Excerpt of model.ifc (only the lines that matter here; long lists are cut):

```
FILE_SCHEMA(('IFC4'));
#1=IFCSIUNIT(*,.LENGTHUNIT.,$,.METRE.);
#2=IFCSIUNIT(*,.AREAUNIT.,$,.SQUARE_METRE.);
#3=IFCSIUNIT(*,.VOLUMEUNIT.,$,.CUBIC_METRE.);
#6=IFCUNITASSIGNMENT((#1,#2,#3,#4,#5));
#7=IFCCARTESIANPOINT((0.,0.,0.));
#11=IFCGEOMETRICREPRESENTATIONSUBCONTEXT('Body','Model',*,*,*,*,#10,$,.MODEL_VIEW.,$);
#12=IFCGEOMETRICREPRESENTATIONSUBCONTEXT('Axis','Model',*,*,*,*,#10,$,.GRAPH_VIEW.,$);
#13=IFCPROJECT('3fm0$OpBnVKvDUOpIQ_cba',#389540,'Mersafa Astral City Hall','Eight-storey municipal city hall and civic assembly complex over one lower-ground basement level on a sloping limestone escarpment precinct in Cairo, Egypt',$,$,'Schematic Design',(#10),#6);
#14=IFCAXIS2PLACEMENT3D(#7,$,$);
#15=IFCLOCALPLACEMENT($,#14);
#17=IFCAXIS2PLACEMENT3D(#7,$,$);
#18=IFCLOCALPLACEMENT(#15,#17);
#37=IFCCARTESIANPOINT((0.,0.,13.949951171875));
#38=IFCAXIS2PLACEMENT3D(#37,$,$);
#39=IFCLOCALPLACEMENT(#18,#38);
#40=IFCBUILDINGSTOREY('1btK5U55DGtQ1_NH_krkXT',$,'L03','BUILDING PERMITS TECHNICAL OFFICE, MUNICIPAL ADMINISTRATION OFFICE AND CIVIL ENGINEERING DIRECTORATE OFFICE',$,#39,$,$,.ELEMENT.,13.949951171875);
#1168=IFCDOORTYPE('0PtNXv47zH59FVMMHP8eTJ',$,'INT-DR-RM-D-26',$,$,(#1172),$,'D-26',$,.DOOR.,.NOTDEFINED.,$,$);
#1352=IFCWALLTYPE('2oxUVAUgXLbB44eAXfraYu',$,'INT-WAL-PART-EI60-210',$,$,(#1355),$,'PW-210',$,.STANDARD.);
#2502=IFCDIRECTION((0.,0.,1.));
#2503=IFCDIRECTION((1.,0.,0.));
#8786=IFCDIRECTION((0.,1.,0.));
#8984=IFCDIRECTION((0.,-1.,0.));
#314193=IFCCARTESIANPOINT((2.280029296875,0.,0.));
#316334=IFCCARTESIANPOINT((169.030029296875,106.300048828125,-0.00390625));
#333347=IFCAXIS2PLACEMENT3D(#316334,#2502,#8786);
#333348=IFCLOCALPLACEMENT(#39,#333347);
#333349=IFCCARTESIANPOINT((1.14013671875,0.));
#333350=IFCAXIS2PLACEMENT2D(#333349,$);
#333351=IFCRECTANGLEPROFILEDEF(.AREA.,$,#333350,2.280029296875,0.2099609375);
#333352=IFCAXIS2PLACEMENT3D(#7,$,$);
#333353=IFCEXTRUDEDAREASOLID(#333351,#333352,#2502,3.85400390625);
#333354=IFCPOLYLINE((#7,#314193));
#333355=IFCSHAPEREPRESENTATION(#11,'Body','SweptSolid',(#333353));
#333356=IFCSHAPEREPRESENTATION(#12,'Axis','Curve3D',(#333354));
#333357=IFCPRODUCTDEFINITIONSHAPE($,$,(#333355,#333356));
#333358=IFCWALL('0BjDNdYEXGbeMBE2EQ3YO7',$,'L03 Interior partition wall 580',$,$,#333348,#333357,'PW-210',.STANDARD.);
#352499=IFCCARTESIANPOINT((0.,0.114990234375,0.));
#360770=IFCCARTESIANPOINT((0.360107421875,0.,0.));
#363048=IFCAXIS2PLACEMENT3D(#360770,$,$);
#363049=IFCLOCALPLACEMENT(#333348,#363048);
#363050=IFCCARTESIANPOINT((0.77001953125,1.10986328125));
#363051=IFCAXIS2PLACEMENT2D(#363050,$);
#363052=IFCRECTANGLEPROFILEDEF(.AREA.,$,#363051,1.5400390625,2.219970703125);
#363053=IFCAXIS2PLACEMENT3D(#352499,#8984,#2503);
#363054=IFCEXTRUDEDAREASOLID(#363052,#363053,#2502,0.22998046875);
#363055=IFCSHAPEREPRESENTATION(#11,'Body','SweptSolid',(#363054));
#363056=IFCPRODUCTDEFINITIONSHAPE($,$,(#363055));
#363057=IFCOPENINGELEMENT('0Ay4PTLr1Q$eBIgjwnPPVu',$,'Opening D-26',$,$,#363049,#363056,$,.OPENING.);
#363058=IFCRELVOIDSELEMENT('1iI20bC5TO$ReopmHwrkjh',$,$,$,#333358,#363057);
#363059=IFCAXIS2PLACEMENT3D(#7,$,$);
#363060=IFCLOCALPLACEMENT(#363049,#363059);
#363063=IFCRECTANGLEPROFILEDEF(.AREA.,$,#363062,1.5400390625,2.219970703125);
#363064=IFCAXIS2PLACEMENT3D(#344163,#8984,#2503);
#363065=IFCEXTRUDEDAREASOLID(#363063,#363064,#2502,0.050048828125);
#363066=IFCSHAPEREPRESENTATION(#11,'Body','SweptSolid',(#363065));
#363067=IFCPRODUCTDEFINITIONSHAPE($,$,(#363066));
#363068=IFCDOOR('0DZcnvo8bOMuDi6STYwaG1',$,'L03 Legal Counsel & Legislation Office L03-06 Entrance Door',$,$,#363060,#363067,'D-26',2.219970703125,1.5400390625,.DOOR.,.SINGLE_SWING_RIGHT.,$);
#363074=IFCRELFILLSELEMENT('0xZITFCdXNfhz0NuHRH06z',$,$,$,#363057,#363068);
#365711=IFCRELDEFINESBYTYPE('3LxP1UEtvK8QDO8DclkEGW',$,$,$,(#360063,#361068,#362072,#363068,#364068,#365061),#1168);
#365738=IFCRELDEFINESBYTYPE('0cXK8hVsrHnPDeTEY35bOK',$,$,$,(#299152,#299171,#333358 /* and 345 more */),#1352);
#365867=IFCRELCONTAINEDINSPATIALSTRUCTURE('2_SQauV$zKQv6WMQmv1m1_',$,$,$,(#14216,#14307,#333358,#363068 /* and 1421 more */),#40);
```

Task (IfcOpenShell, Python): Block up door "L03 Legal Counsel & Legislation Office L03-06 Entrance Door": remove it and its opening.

```python
import ifcopenshell
import ifcopenshell.api.feature
import ifcopenshell.api.root
import ifcopenshell.geom
import ifcopenshell.util.shape

model = ifcopenshell.open("model.ifc")
settings = ifcopenshell.geom.settings()


def volume(element):
    """Net volume in cubic metres, openings subtracted."""
    shape = ifcopenshell.geom.create_shape(settings, element)
    return ifcopenshell.util.shape.get_volume(shape.geometry)


door = model.by_guid("0DZcnvo8bOMuDi6STYwaG1")
opening = door.FillsVoids[0].RelatingOpeningElement
wall = opening.VoidsElements[0].RelatingBuildingElement
before = volume(wall)

ifcopenshell.api.root.remove_product(model, product=door)
ifcopenshell.api.feature.remove_feature(model, feature=opening)

after = volume(wall)

print(f"wall volume {before:.3f} -> {after:.3f} m3")

model.write("model_rev.ifc")
```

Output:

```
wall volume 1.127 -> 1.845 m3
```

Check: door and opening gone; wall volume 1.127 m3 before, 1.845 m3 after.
